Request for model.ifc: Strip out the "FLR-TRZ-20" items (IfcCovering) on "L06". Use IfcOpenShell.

First a look at what the model holds.

```python
import ifcopenshell
import ifcopenshell.util.element

model = ifcopenshell.open("model.ifc")
print(model.schema)
storey = next(s for s in model.by_type("IfcBuildingStorey") if s.Name == "L06")
coverings = [e for e in ifcopenshell.util.element.get_decomposition(storey) if e.is_a("IfcCovering")]
seen = {}
for e in coverings:
    element_type = ifcopenshell.util.element.get_type(e)
    name = element_type.Name if element_type not in (None, e) else None
    seen[name] = seen.get(name, 0) + 1
for name, count in sorted(seen.items(), key=str):
    print(count, "x", name)
```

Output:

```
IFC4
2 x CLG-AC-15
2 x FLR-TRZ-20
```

```python
import ifcopenshell
import ifcopenshell.api.root
import ifcopenshell.util.element

model = ifcopenshell.open("model.ifc")

storey = next(s for s in model.by_type("IfcBuildingStorey") if s.Name == "L06")
coverings = [e for e in ifcopenshell.util.element.get_decomposition(storey) if e.is_a("IfcCovering")]
targets = [e for e in coverings if (t := ifcopenshell.util.element.get_type(e)) not in (None, e) and t.Name == "FLR-TRZ-20"]

for e in targets:
    ifcopenshell.api.root.remove_product(model, product=e)
print(len(targets), "removed")

model.write("model_v2.ifc")
```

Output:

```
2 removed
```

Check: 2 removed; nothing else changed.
